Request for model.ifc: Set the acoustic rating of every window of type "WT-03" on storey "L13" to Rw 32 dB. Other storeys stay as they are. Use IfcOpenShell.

First a look at what the model holds.

```python
import ifcopenshell
import ifcopenshell.util.element

model = ifcopenshell.open("model.ifc")
print(model.schema)
storey = next(s for s in model.by_type("IfcBuildingStorey") if s.Name == "L13")
windows = [e for e in ifcopenshell.util.element.get_decomposition(storey) if e.is_a("IfcWindow")]
seen = {}
for e in windows:
    element_type = ifcopenshell.util.element.get_type(e)
    key = (element_type.Name if element_type != e and element_type else None, ifcopenshell.util.element.get_pset(e, "Pset_WindowCommon", "AcousticRating"))
    seen[key] = seen.get(key, 0) + 1
for (name, value), count in sorted(seen.items(), key=str):
    print(count, "x", name, "|", value)
```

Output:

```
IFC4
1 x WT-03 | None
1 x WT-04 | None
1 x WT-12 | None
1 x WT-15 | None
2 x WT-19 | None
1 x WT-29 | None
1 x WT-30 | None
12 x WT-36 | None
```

```python
import ifcopenshell
import ifcopenshell.api.pset
import ifcopenshell.util.element

model = ifcopenshell.open("model.ifc")

storey = next(s for s in model.by_type("IfcBuildingStorey") if s.Name == "L13")
windows = [e for e in ifcopenshell.util.element.get_decomposition(storey) if e.is_a("IfcWindow")]

count = 0
for e in windows:
    element_type = ifcopenshell.util.element.get_type(e)
    if element_type in (None, e) or element_type.Name != "WT-03":
        continue
    # add_pset returns the element's existing set when there is one.
    pset = ifcopenshell.api.pset.add_pset(model, product=e, name="Pset_WindowCommon")
    ifcopenshell.api.pset.edit_pset(model, pset=pset, properties={"AcousticRating": "Rw 32 dB"})
    count += 1

print(count, "windows updated")

model.write("model_v2.ifc")
```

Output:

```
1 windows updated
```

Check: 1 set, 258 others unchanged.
